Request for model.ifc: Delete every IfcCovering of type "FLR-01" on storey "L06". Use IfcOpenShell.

First a look at what the model holds.

```python
import ifcopenshell
import ifcopenshell.util.element

model = ifcopenshell.open("model.ifc")
print(model.schema)
storey = next(s for s in model.by_type("IfcBuildingStorey") if s.Name == "L06")
coverings = [e for e in ifcopenshell.util.element.get_decomposition(storey) if e.is_a("IfcCovering")]
seen = {}
for e in coverings:
    element_type = ifcopenshell.util.element.get_type(e)
    name = element_type.Name if element_type not in (None, e) else None
    seen[name] = seen.get(name, 0) + 1
for name, count in sorted(seen.items(), key=str):
    print(count, "x", name)
```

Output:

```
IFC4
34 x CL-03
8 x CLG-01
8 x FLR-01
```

```python
import ifcopenshell
import ifcopenshell.api.root
import ifcopenshell.util.element

model = ifcopenshell.open("model.ifc")

storey = next(s for s in model.by_type("IfcBuildingStorey") if s.Name == "L06")
coverings = [e for e in ifcopenshell.util.element.get_decomposition(storey) if e.is_a("IfcCovering")]
targets = [e for e in coverings if (t := ifcopenshell.util.element.get_type(e)) not in (None, e) and t.Name == "FLR-01"]

for e in targets:
    ifcopenshell.api.root.remove_product(model, product=e)
print(len(targets), "removed")

model.write("model_rev.ifc")
```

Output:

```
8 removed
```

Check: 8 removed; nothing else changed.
